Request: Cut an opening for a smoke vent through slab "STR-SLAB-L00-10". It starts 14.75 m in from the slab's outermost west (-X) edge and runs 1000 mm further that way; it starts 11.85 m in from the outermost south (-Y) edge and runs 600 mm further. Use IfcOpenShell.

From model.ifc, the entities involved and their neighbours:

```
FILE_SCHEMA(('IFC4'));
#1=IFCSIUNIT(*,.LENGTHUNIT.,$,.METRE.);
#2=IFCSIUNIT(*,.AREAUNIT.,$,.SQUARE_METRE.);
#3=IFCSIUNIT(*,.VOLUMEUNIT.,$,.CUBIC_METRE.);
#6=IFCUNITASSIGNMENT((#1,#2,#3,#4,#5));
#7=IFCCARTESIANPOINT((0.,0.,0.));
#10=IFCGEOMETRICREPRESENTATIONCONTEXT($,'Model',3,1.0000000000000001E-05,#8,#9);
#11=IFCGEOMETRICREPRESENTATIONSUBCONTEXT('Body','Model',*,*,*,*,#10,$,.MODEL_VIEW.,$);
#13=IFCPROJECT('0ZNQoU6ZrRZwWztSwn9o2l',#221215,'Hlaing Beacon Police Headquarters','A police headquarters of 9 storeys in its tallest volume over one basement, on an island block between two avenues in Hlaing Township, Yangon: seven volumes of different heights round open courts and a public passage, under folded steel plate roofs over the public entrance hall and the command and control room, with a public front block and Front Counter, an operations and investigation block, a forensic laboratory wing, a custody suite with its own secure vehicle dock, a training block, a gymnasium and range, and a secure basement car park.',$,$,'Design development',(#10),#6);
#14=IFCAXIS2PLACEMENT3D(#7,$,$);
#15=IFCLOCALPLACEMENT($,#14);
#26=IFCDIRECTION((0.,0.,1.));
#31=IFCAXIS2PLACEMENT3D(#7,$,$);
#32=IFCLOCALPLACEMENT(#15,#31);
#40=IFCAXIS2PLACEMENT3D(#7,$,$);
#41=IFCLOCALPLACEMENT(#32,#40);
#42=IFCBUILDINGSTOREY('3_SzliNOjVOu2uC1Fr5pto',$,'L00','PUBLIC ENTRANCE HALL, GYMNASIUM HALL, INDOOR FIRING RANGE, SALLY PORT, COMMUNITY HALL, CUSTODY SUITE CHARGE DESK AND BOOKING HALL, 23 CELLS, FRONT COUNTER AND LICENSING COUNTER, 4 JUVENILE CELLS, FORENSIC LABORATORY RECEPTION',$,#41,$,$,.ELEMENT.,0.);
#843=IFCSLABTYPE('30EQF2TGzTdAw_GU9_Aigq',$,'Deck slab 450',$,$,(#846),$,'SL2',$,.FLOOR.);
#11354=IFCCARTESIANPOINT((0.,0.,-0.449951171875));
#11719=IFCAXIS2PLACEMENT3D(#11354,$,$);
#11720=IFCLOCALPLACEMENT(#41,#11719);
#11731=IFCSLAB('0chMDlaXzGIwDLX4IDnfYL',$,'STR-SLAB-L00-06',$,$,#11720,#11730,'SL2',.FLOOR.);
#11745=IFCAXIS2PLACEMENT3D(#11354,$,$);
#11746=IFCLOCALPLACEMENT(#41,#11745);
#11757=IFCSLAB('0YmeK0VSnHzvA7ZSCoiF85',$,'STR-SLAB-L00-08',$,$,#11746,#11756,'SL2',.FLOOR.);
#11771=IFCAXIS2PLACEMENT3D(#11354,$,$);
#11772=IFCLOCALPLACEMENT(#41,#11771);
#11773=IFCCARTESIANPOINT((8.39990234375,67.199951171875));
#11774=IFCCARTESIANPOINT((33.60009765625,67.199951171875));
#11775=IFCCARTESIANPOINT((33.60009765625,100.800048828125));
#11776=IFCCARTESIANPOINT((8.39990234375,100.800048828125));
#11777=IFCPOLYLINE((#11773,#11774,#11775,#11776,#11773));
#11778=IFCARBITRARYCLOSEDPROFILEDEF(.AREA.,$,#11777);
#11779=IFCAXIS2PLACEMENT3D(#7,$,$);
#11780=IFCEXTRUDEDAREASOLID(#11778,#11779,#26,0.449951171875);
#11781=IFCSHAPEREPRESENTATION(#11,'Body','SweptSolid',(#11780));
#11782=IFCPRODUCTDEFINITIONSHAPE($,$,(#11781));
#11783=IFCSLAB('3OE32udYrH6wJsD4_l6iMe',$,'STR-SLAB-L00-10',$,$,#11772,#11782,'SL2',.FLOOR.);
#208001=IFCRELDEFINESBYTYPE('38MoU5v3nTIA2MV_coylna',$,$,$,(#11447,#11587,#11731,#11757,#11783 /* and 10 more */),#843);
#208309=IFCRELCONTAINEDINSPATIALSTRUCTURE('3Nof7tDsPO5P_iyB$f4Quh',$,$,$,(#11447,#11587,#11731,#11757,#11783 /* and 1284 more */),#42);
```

```python
import numpy as np
import ifcopenshell
import ifcopenshell.api.feature
import ifcopenshell.api.geometry
import ifcopenshell.api.root
import ifcopenshell.geom
import ifcopenshell.util.placement
import ifcopenshell.util.representation
import ifcopenshell.util.shape
import ifcopenshell.util.unit

model = ifcopenshell.open("model.ifc")
unit_scale = ifcopenshell.util.unit.calculate_unit_scale(model)
settings = ifcopenshell.geom.settings()


def volume(element):
    """Net volume in cubic metres, openings subtracted."""
    shape = ifcopenshell.geom.create_shape(settings, element)
    return ifcopenshell.util.shape.get_volume(shape.geometry)


slab = model.by_guid("3OE32udYrH6wJsD4_l6iMe")
before = volume(slab)

# Extent in the slab's own axes, in metres. The edges named are its -X and -Y sides.
slab_shape = ifcopenshell.geom.create_shape(settings, slab)
vertices = ifcopenshell.util.shape.get_vertices(slab_shape.geometry)
x_min, y_min, bottom = vertices.min(axis=0)
top = vertices[:, 2].max()

opening = ifcopenshell.api.root.create_entity(model, ifc_class="IfcOpeningElement", name="Smoke vent opening", predefined_type="OPENING")
context = ifcopenshell.util.representation.get_context(model, "Model", "Body", "MODEL_VIEW")
width, depth = 1, 0.6
outline = [(0.0, 0.0), (width, 0.0), (width, depth), (0.0, depth), (0.0, 0.0)]
# Overshoot both faces by 50 mm so the cut is clean.
shape = ifcopenshell.api.geometry.add_slab_representation(
    model, context=context, depth=top - bottom + 0.1, polyline=outline
)
ifcopenshell.api.geometry.assign_representation(model, product=opening, representation=shape)

matrix = ifcopenshell.util.placement.get_local_placement(slab.ObjectPlacement)
matrix[:, 3] = matrix @ np.append(np.array([x_min + 14.75, y_min + 11.85, bottom - 0.05]) / unit_scale, 1.0)
ifcopenshell.api.geometry.edit_object_placement(model, product=opening, matrix=matrix, is_si=False)
ifcopenshell.api.feature.add_feature(model, feature=opening, element=slab)

after = volume(slab)

print(f"slab volume {before:.3f} -> {after:.3f} m3")

model.write("model_updated.ifc")
```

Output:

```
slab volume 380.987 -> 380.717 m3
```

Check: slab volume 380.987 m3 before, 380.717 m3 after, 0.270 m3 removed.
